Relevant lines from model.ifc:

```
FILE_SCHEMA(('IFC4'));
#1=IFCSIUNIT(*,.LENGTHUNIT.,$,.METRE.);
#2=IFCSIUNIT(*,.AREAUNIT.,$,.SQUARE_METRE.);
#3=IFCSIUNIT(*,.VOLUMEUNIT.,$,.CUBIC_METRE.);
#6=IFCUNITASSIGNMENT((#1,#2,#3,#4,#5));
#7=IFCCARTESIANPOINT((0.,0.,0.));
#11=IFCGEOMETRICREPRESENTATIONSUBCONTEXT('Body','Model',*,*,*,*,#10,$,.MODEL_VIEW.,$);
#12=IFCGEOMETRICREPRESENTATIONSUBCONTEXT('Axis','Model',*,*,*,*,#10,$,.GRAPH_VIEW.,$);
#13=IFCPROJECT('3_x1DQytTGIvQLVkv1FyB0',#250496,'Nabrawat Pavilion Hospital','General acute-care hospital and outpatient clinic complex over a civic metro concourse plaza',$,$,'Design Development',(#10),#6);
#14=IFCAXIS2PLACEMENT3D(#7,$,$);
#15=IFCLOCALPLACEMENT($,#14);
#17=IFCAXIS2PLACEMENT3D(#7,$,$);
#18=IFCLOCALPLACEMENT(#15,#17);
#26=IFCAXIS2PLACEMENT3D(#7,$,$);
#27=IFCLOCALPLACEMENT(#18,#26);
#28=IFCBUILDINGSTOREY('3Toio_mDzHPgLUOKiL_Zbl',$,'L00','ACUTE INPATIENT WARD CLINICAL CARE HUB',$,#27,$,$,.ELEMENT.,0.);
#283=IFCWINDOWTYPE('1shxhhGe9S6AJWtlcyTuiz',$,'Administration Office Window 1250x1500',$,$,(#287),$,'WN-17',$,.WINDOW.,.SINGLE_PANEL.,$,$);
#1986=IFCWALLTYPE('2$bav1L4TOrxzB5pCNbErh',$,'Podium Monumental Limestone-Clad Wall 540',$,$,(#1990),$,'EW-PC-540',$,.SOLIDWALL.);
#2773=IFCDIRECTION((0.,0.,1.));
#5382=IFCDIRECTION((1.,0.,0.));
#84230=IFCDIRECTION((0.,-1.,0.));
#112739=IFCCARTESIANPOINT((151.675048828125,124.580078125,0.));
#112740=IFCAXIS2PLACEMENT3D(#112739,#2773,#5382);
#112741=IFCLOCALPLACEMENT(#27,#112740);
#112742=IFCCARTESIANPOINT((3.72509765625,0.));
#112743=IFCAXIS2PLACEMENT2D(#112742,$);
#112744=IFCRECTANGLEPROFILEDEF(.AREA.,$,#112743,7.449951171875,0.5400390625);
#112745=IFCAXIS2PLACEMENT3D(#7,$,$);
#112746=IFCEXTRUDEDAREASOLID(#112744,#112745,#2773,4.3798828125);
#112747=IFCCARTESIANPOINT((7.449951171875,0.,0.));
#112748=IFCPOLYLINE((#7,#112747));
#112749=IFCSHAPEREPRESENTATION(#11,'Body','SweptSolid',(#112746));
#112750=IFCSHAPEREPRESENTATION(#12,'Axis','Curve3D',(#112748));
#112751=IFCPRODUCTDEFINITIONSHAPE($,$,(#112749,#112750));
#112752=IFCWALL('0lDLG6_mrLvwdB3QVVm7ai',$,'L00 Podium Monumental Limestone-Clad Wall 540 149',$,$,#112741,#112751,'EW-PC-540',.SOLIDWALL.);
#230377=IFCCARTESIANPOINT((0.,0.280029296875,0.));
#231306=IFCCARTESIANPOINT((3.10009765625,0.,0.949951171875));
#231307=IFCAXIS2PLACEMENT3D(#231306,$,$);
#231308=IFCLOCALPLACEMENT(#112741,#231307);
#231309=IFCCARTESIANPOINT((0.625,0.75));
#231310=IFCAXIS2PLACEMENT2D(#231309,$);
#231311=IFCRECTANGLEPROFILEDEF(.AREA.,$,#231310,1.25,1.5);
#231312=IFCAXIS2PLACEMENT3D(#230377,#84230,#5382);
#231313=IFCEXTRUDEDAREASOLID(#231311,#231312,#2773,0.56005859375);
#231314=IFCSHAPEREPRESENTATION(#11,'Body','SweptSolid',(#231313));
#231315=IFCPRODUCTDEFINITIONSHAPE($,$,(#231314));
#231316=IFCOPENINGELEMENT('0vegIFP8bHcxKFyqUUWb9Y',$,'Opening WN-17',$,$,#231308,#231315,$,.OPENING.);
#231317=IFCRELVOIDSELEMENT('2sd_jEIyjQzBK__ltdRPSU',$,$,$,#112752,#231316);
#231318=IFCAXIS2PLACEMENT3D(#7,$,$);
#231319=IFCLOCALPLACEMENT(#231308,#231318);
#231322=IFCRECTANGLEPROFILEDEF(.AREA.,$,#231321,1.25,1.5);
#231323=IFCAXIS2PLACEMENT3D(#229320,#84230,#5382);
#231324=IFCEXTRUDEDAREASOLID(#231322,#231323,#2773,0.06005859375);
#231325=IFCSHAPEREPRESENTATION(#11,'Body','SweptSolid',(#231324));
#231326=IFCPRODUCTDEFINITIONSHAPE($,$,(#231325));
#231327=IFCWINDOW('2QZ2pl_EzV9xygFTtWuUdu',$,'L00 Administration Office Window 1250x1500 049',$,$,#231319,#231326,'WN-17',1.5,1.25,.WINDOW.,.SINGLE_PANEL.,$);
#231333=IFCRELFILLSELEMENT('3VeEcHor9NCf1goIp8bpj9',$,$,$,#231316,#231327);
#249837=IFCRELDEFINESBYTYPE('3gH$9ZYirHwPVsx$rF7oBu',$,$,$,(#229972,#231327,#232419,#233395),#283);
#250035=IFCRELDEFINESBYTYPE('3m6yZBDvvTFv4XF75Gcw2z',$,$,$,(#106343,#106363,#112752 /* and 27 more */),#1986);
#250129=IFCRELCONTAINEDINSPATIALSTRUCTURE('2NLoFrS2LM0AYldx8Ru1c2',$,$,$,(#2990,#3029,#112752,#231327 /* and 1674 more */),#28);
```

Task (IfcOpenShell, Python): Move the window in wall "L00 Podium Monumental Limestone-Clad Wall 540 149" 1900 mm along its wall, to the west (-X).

```python
import ifcopenshell
import ifcopenshell.api.geometry
import ifcopenshell.util.placement
import ifcopenshell.util.unit

model = ifcopenshell.open("model.ifc")
unit_scale = ifcopenshell.util.unit.calculate_unit_scale(model)

window = model.by_guid("2QZ2pl_EzV9xygFTtWuUdu")
opening = window.FillsVoids[0].RelatingOpeningElement
wall = opening.VoidsElements[0].RelatingBuildingElement

wall_matrix = ifcopenshell.util.placement.get_local_placement(wall.ObjectPlacement)
shift = wall_matrix[:3, 0] * -1.9 / unit_scale
before = ifcopenshell.util.placement.get_local_placement(window.ObjectPlacement)[:3, 3].copy()

# The window is placed relative to its opening, so it follows when the opening moves.
matrix = ifcopenshell.util.placement.get_local_placement(opening.ObjectPlacement)
matrix[:3, 3] += shift
ifcopenshell.api.geometry.edit_object_placement(
    model, product=opening, matrix=matrix, is_si=False, should_transform_children=True
)

after = ifcopenshell.util.placement.get_local_placement(window.ObjectPlacement)[:3, 3]
print("window moved by", (after - before).round(3) + 0.0)

model.write("model-out.ifc")
```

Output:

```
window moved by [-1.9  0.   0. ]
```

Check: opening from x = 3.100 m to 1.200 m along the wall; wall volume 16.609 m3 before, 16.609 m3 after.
